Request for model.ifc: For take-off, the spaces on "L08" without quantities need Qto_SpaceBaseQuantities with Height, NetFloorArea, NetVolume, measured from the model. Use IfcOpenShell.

First a look at what the model holds.

```python
import ifcopenshell
import ifcopenshell.util.element
import ifcopenshell.util.unit

model = ifcopenshell.open("model.ifc")
print(model.schema)
for unit_type in ("LENGTHUNIT", "AREAUNIT", "VOLUMEUNIT"):
    print(unit_type, ifcopenshell.util.unit.calculate_unit_scale(model, unit_type))
storey = next(s for s in model.by_type("IfcBuildingStorey") if s.Name == "L08")
spaces = [e for e in ifcopenshell.util.element.get_decomposition(storey) if e.is_a("IfcSpace")]
for e in sorted(spaces, key=lambda e: e.id()):
    print(e.id(), e.is_a(), e.Name, list(ifcopenshell.util.element.get_psets(e, qtos_only=True)), sep=" | ")
```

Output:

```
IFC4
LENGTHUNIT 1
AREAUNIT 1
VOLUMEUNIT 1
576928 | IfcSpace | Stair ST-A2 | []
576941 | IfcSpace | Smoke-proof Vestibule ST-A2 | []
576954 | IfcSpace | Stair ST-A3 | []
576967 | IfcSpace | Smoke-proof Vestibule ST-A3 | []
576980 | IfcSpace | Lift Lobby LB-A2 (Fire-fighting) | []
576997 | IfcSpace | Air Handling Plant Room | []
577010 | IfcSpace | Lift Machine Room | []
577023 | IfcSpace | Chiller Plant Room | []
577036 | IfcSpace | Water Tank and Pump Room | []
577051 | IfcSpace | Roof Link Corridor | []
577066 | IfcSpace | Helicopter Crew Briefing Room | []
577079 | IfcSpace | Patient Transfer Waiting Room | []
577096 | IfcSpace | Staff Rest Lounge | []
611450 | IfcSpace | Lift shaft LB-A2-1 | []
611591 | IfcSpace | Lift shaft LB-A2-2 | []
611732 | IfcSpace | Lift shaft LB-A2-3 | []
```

```python
import ifcopenshell
import ifcopenshell.api.pset
import ifcopenshell.geom
import ifcopenshell.util.element
import ifcopenshell.util.shape
import ifcopenshell.util.unit

model = ifcopenshell.open("model.ifc")
unit_scale = ifcopenshell.util.unit.calculate_unit_scale(model)
area_scale = ifcopenshell.util.unit.calculate_unit_scale(model, "AREAUNIT")
volume_scale = ifcopenshell.util.unit.calculate_unit_scale(model, "VOLUMEUNIT")
settings = ifcopenshell.geom.settings()

storey = next(s for s in model.by_type("IfcBuildingStorey") if s.Name == "L08")
spaces = [e for e in ifcopenshell.util.element.get_decomposition(storey) if e.is_a("IfcSpace")]

for e in sorted(spaces, key=lambda e: e.id()):
    if ifcopenshell.util.element.get_psets(e, qtos_only=True, should_inherit=False):
        continue
    # Geometry comes back in metres, in the element's own axes.
    shape = ifcopenshell.geom.create_shape(settings, e)
    values = {
        "Height": ifcopenshell.util.shape.get_z(shape.geometry) / unit_scale,
        "NetFloorArea": ifcopenshell.util.shape.get_footprint_area(shape.geometry) / area_scale,
        "NetVolume": ifcopenshell.util.shape.get_volume(shape.geometry) / volume_scale,
    }
    qto = ifcopenshell.api.pset.add_qto(model, product=e, name="Qto_SpaceBaseQuantities")
    ifcopenshell.api.pset.edit_qto(model, qto=qto, properties=values)
    print(e.id(), {k: round(v, 3) for k, v in values.items()})

model.write("model_v2.ifc")
```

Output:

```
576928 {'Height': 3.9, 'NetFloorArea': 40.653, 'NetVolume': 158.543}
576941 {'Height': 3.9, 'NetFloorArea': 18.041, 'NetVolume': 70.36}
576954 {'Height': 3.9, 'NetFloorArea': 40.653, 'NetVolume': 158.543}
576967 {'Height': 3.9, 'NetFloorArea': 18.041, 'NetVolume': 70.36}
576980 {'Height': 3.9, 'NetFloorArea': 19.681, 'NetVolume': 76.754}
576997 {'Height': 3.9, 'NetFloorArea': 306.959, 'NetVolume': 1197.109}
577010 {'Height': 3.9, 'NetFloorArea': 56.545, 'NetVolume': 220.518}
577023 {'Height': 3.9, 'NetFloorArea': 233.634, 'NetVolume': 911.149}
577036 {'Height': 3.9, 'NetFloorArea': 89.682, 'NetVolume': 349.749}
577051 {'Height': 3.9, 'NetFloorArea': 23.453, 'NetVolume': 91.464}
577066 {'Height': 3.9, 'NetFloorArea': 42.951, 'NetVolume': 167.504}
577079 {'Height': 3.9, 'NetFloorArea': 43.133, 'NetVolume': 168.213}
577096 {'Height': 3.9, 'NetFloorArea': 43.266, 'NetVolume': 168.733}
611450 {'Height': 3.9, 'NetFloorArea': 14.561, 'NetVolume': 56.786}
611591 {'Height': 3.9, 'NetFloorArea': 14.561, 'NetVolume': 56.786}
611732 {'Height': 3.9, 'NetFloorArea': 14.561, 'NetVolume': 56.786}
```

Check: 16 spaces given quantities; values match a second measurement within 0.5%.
